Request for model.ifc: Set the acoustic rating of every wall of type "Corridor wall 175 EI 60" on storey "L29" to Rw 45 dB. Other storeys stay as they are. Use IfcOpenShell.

First a look at what the model holds.

```python
import ifcopenshell
import ifcopenshell.util.element

model = ifcopenshell.open("model.ifc")
print(model.schema)
storey = next(s for s in model.by_type("IfcBuildingStorey") if s.Name == "L29")
walls = [e for e in ifcopenshell.util.element.get_decomposition(storey) if e.is_a("IfcWall")]
seen = {}
for e in walls:
    element_type = ifcopenshell.util.element.get_type(e)
    key = (element_type.Name if element_type != e and element_type else None, ifcopenshell.util.element.get_pset(e, "Pset_WallCommon", "AcousticRating"))
    seen[key] = seen.get(key, 0) + 1
for (name, value), count in sorted(seen.items(), key=str):
    print(count, "x", name, "|", value)
```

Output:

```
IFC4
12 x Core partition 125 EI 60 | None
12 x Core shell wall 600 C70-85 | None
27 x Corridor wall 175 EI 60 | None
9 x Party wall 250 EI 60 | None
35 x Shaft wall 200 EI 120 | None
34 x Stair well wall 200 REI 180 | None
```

```python
import ifcopenshell
import ifcopenshell.api.pset
import ifcopenshell.util.element

model = ifcopenshell.open("model.ifc")

storey = next(s for s in model.by_type("IfcBuildingStorey") if s.Name == "L29")
walls = [e for e in ifcopenshell.util.element.get_decomposition(storey) if e.is_a("IfcWall")]

count = 0
for e in walls:
    element_type = ifcopenshell.util.element.get_type(e)
    if element_type in (None, e) or element_type.Name != "Corridor wall 175 EI 60":
        continue
    found = ifcopenshell.util.element.get_pset(e, "Pset_WallCommon", should_inherit=False)
    if found:
        pset = model.by_id(found["id"])
        if len(ifcopenshell.util.element.get_elements_by_pset(pset)) > 1:
            pset = ifcopenshell.api.pset.unshare_pset(model, products=[e], pset=pset)[0]
    else:
        pset = ifcopenshell.api.pset.add_pset(model, product=e, name="Pset_WallCommon")
    ifcopenshell.api.pset.edit_pset(model, pset=pset, properties={"AcousticRating": "Rw 45 dB"})
    count += 1

print(count, "walls updated")

model.write("model_updated.ifc")
```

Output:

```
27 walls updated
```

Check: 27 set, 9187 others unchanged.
